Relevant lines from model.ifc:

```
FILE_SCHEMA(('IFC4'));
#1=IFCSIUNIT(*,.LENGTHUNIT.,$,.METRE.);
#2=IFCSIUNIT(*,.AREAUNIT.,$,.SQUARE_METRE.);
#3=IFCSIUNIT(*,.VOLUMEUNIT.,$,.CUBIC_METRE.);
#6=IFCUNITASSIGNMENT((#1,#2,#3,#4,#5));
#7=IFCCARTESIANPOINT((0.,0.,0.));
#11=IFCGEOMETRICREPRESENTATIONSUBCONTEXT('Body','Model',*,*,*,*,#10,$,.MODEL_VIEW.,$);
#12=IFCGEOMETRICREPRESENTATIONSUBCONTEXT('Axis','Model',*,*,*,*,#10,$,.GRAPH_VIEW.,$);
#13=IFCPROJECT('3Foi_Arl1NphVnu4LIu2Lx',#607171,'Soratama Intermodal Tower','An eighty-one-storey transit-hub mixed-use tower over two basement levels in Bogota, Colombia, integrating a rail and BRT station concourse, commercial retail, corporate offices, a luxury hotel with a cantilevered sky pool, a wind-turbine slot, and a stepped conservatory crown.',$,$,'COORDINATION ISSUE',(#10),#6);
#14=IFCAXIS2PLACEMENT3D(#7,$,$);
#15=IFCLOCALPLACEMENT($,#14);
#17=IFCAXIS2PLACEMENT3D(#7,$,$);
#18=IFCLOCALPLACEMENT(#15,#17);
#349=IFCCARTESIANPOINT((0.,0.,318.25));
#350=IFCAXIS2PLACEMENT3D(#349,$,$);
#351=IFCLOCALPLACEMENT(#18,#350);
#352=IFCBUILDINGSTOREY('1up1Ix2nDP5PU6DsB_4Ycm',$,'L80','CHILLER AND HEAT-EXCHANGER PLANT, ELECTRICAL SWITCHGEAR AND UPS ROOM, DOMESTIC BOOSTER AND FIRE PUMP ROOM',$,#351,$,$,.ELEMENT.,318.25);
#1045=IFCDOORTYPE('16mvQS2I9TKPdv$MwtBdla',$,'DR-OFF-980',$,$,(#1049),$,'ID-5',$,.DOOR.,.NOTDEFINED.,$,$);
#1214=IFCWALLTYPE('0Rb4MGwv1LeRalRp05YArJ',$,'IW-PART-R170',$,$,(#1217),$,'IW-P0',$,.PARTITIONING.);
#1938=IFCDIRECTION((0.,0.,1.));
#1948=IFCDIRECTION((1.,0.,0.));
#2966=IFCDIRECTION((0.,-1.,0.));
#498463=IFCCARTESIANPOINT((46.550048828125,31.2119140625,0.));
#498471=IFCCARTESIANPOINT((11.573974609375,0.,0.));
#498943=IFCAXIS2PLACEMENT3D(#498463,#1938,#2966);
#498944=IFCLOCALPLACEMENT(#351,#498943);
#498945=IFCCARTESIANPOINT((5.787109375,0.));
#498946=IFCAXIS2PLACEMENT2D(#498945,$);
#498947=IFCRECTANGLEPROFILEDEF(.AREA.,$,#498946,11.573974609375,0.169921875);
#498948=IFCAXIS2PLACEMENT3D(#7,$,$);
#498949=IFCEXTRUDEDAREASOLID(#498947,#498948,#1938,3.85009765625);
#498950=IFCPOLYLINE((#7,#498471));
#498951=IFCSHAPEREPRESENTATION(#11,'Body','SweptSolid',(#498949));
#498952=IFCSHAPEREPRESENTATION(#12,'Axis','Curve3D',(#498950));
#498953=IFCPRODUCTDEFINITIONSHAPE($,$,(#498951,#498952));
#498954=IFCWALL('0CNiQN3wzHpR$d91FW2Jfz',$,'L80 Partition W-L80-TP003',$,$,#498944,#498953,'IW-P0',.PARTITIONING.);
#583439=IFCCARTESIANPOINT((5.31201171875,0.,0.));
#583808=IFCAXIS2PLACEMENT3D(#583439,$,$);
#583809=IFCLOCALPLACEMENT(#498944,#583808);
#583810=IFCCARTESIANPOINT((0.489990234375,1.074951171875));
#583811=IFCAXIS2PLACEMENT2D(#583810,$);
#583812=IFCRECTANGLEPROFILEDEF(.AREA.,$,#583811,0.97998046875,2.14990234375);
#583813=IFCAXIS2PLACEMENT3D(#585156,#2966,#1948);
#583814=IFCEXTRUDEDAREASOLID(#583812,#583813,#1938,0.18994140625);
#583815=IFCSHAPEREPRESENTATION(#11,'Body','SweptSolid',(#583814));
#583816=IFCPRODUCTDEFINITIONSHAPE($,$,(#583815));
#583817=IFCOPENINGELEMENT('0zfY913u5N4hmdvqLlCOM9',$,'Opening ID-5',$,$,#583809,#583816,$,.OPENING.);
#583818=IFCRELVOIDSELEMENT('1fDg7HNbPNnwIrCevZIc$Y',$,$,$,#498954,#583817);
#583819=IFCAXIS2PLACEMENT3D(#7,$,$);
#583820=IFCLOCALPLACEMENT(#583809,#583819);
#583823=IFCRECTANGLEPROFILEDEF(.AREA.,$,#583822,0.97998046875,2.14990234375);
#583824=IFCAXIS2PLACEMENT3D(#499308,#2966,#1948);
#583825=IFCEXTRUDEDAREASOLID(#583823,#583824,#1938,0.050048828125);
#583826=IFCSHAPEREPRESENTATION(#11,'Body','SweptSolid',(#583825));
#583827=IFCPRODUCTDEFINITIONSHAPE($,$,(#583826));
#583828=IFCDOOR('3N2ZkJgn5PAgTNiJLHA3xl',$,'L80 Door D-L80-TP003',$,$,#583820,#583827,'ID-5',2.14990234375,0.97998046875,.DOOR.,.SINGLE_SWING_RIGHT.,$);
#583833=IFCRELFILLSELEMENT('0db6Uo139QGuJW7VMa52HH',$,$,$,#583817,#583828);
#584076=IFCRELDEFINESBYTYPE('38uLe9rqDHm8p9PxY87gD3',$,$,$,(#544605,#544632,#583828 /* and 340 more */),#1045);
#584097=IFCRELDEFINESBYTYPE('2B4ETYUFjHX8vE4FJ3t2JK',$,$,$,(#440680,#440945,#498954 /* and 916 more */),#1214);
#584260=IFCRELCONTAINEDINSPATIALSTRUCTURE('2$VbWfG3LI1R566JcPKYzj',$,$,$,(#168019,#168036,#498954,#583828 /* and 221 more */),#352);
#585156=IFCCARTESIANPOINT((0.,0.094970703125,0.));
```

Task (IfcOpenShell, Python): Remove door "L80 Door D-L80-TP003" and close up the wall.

```python
import ifcopenshell
import ifcopenshell.api.feature
import ifcopenshell.api.root
import ifcopenshell.geom
import ifcopenshell.util.shape

model = ifcopenshell.open("model.ifc")
settings = ifcopenshell.geom.settings()


def volume(element):
    """Net volume in cubic metres, openings subtracted."""
    shape = ifcopenshell.geom.create_shape(settings, element)
    return ifcopenshell.util.shape.get_volume(shape.geometry)


door = model.by_id(583828)
opening = door.FillsVoids[0].RelatingOpeningElement
wall = opening.VoidsElements[0].RelatingBuildingElement
before = volume(wall)

ifcopenshell.api.root.remove_product(model, product=door)
ifcopenshell.api.feature.remove_feature(model, feature=opening)

after = volume(wall)

print(f"wall volume {before:.3f} -> {after:.3f} m3")

model.write("model_edited.ifc")
```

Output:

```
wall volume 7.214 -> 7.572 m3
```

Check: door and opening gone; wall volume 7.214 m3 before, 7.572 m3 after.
